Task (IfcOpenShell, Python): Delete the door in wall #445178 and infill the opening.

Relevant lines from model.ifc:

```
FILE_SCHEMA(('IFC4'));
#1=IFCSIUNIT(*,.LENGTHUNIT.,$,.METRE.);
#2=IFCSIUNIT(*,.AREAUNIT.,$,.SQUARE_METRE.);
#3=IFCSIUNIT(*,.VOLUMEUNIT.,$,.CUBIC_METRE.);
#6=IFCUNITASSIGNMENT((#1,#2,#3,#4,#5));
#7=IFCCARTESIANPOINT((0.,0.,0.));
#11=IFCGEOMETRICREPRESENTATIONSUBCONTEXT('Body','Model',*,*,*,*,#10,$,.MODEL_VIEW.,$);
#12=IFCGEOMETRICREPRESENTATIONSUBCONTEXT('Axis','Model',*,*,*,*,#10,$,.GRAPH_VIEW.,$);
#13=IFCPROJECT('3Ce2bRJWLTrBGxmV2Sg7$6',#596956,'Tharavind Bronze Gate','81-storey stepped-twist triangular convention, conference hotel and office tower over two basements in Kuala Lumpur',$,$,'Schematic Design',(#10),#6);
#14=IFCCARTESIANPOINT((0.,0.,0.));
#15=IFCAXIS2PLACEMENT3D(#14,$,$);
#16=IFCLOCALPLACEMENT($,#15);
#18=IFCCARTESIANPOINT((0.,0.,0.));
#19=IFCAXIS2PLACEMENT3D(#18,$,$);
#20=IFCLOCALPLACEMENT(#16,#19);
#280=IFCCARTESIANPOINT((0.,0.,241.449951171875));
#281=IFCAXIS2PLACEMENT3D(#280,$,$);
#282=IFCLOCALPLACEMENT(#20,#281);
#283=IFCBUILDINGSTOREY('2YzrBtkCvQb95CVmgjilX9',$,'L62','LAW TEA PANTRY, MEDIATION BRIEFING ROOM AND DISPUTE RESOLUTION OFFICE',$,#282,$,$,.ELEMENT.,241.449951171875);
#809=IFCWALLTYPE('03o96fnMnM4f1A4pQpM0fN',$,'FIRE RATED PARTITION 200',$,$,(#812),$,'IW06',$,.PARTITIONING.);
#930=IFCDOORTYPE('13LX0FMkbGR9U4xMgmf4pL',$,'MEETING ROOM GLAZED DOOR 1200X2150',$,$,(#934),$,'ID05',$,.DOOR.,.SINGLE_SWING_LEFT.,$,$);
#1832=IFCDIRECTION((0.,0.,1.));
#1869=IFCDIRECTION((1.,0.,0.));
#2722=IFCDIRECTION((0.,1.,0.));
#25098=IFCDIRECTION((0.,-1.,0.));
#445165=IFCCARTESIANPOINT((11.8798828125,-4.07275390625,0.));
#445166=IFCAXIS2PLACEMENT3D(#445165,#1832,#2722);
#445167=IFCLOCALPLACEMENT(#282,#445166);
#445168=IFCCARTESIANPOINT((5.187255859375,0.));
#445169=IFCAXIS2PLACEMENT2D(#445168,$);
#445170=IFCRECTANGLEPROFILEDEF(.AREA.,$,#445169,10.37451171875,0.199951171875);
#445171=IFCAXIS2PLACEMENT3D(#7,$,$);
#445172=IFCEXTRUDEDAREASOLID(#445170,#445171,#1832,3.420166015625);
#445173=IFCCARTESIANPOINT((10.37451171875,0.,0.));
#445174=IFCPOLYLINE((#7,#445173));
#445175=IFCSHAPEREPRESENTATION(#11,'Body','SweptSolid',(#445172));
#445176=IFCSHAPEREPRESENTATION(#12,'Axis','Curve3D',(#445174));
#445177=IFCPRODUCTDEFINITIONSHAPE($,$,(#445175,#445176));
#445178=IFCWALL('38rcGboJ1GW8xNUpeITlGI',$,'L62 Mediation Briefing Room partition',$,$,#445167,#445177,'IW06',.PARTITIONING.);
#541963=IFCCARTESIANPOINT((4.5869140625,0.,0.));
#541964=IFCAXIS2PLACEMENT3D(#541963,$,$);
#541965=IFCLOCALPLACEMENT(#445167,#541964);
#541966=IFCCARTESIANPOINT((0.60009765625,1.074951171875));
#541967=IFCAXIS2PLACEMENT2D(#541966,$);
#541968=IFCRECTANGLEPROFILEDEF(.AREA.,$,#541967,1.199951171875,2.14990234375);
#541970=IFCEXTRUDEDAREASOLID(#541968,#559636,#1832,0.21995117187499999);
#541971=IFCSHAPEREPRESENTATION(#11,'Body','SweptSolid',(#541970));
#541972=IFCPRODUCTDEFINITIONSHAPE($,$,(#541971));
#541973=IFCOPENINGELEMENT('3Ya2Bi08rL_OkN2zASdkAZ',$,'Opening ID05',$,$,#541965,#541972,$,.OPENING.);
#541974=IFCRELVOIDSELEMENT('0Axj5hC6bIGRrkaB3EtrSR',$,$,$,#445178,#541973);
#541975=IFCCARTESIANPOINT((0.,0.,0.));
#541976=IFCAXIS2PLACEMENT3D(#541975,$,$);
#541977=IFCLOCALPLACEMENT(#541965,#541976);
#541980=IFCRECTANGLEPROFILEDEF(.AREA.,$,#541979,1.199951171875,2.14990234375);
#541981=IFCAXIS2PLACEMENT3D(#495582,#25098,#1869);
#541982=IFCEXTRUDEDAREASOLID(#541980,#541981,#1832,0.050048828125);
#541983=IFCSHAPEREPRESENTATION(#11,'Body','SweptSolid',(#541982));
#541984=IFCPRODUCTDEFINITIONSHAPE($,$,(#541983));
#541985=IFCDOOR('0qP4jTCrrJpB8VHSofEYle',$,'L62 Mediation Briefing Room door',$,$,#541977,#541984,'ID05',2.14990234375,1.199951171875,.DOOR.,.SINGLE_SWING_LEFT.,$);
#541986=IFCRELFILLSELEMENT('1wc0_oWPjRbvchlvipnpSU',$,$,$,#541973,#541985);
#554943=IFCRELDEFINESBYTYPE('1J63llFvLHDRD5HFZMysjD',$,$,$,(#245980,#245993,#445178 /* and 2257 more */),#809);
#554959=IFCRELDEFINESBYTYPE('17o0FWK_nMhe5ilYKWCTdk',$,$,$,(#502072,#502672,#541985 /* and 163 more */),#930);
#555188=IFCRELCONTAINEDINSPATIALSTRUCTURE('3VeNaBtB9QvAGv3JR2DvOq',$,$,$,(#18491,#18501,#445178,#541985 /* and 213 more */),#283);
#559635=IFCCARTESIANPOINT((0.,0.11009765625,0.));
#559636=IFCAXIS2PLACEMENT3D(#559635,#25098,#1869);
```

```python
import ifcopenshell
import ifcopenshell.api.feature
import ifcopenshell.api.root
import ifcopenshell.geom
import ifcopenshell.util.shape

model = ifcopenshell.open("model.ifc")
settings = ifcopenshell.geom.settings()


def volume(element):
    """Net volume in cubic metres, openings subtracted."""
    shape = ifcopenshell.geom.create_shape(settings, element)
    return ifcopenshell.util.shape.get_volume(shape.geometry)


door = model.by_guid("0qP4jTCrrJpB8VHSofEYle")
opening = door.FillsVoids[0].RelatingOpeningElement
wall = opening.VoidsElements[0].RelatingBuildingElement
before = volume(wall)

ifcopenshell.api.root.remove_product(model, product=door)
ifcopenshell.api.feature.remove_feature(model, feature=opening)

after = volume(wall)

print(f"wall volume {before:.3f} -> {after:.3f} m3")

model.write("model_v2.ifc")
```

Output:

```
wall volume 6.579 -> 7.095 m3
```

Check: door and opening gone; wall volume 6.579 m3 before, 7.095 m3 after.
